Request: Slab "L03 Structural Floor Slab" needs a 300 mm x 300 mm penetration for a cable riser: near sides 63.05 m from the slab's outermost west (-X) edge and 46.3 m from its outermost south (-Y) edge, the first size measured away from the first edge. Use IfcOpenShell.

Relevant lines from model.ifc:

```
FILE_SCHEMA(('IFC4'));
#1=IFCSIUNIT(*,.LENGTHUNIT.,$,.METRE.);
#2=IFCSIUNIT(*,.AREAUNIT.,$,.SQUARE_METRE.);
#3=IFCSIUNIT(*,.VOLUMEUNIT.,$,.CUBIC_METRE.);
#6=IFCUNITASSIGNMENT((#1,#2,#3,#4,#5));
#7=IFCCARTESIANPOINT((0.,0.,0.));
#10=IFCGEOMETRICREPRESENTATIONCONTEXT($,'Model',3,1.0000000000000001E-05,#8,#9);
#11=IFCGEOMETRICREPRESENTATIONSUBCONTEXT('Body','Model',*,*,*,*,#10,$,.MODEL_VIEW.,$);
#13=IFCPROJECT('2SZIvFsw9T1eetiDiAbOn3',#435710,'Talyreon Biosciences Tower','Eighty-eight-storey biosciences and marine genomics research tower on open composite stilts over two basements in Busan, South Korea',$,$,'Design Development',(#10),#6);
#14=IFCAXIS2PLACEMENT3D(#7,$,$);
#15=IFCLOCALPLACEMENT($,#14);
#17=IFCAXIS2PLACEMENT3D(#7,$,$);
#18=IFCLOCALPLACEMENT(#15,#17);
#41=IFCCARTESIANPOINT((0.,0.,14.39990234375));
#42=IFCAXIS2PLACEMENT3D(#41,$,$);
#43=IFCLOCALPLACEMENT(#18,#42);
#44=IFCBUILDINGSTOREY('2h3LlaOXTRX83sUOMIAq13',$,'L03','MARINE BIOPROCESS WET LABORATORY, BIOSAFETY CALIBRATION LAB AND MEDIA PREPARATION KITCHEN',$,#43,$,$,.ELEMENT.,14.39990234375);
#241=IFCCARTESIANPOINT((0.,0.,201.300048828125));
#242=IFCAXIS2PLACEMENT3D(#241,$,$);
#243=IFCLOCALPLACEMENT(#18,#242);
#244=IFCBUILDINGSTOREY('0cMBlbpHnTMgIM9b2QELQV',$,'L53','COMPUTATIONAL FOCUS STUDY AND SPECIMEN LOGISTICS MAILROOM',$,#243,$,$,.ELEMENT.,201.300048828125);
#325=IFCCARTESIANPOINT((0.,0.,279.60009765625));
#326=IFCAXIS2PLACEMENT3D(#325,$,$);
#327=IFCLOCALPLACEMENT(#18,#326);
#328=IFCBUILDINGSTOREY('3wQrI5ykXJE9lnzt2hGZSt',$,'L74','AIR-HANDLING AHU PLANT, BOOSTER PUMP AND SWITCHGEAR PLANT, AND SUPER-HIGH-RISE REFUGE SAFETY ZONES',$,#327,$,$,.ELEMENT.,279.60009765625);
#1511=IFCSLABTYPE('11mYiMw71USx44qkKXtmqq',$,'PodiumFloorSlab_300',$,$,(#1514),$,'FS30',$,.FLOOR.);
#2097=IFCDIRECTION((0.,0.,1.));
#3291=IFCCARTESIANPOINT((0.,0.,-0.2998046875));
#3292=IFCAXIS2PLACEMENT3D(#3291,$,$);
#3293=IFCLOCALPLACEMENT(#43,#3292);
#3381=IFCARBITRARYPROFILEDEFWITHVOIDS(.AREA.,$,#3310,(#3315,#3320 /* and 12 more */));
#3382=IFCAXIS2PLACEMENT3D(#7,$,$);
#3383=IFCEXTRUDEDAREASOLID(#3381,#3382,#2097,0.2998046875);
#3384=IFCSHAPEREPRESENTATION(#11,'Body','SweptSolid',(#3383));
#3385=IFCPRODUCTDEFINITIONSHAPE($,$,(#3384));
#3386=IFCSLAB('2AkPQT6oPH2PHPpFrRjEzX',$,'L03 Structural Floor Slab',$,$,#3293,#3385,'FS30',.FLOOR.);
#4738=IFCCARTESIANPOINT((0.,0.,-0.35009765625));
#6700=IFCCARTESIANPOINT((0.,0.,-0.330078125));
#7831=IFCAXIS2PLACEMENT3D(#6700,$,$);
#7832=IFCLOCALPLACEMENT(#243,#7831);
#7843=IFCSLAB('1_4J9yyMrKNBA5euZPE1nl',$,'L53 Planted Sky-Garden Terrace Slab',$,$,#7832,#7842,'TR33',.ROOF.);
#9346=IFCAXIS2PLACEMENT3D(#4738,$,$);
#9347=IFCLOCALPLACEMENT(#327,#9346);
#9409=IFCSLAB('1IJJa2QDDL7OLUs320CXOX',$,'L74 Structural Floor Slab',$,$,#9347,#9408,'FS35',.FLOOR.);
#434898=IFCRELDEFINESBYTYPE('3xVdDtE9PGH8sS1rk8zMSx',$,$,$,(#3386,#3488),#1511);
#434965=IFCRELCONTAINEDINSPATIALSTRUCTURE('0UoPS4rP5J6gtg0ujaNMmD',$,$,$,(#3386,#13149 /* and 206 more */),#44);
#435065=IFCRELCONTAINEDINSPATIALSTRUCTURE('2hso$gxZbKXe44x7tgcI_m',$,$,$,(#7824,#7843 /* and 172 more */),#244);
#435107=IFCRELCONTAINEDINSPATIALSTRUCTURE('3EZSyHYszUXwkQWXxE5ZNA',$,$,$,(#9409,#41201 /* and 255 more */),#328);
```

```python
import numpy as np
import ifcopenshell
import ifcopenshell.api.feature
import ifcopenshell.api.geometry
import ifcopenshell.api.root
import ifcopenshell.geom
import ifcopenshell.util.placement
import ifcopenshell.util.representation
import ifcopenshell.util.shape
import ifcopenshell.util.unit

model = ifcopenshell.open("model.ifc")
unit_scale = ifcopenshell.util.unit.calculate_unit_scale(model)
settings = ifcopenshell.geom.settings()


def volume(element):
    """Net volume in cubic metres, openings subtracted."""
    shape = ifcopenshell.geom.create_shape(settings, element)
    return ifcopenshell.util.shape.get_volume(shape.geometry)


slab = model.by_guid("2AkPQT6oPH2PHPpFrRjEzX")
before = volume(slab)

# Extent in the slab's own axes, in metres. The edges named are its -X and -Y sides.
slab_shape = ifcopenshell.geom.create_shape(settings, slab)
vertices = ifcopenshell.util.shape.get_vertices(slab_shape.geometry)
x_min, y_min, bottom = vertices.min(axis=0)
top = vertices[:, 2].max()

opening = ifcopenshell.api.root.create_entity(model, ifc_class="IfcOpeningElement", name="Cable riser opening", predefined_type="OPENING")
context = ifcopenshell.util.representation.get_context(model, "Model", "Body", "MODEL_VIEW")
width, depth = 0.3, 0.3
outline = [(0.0, 0.0), (width, 0.0), (width, depth), (0.0, depth), (0.0, 0.0)]
# Overshoot both faces by 50 mm so the cut is clean.
shape = ifcopenshell.api.geometry.add_slab_representation(
    model, context=context, depth=top - bottom + 0.1, polyline=outline
)
ifcopenshell.api.geometry.assign_representation(model, product=opening, representation=shape)

matrix = ifcopenshell.util.placement.get_local_placement(slab.ObjectPlacement)
matrix[:, 3] = matrix @ np.append(np.array([x_min + 63.05, y_min + 46.3, bottom - 0.05]) / unit_scale, 1.0)
ifcopenshell.api.geometry.edit_object_placement(model, product=opening, matrix=matrix, is_si=False)
ifcopenshell.api.feature.add_feature(model, feature=opening, element=slab)

after = volume(slab)

print(f"slab volume {before:.3f} -> {after:.3f} m3")

model.write("model_updated.ifc")
```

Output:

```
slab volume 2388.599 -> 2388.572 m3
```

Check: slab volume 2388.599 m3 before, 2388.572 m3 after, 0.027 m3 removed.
